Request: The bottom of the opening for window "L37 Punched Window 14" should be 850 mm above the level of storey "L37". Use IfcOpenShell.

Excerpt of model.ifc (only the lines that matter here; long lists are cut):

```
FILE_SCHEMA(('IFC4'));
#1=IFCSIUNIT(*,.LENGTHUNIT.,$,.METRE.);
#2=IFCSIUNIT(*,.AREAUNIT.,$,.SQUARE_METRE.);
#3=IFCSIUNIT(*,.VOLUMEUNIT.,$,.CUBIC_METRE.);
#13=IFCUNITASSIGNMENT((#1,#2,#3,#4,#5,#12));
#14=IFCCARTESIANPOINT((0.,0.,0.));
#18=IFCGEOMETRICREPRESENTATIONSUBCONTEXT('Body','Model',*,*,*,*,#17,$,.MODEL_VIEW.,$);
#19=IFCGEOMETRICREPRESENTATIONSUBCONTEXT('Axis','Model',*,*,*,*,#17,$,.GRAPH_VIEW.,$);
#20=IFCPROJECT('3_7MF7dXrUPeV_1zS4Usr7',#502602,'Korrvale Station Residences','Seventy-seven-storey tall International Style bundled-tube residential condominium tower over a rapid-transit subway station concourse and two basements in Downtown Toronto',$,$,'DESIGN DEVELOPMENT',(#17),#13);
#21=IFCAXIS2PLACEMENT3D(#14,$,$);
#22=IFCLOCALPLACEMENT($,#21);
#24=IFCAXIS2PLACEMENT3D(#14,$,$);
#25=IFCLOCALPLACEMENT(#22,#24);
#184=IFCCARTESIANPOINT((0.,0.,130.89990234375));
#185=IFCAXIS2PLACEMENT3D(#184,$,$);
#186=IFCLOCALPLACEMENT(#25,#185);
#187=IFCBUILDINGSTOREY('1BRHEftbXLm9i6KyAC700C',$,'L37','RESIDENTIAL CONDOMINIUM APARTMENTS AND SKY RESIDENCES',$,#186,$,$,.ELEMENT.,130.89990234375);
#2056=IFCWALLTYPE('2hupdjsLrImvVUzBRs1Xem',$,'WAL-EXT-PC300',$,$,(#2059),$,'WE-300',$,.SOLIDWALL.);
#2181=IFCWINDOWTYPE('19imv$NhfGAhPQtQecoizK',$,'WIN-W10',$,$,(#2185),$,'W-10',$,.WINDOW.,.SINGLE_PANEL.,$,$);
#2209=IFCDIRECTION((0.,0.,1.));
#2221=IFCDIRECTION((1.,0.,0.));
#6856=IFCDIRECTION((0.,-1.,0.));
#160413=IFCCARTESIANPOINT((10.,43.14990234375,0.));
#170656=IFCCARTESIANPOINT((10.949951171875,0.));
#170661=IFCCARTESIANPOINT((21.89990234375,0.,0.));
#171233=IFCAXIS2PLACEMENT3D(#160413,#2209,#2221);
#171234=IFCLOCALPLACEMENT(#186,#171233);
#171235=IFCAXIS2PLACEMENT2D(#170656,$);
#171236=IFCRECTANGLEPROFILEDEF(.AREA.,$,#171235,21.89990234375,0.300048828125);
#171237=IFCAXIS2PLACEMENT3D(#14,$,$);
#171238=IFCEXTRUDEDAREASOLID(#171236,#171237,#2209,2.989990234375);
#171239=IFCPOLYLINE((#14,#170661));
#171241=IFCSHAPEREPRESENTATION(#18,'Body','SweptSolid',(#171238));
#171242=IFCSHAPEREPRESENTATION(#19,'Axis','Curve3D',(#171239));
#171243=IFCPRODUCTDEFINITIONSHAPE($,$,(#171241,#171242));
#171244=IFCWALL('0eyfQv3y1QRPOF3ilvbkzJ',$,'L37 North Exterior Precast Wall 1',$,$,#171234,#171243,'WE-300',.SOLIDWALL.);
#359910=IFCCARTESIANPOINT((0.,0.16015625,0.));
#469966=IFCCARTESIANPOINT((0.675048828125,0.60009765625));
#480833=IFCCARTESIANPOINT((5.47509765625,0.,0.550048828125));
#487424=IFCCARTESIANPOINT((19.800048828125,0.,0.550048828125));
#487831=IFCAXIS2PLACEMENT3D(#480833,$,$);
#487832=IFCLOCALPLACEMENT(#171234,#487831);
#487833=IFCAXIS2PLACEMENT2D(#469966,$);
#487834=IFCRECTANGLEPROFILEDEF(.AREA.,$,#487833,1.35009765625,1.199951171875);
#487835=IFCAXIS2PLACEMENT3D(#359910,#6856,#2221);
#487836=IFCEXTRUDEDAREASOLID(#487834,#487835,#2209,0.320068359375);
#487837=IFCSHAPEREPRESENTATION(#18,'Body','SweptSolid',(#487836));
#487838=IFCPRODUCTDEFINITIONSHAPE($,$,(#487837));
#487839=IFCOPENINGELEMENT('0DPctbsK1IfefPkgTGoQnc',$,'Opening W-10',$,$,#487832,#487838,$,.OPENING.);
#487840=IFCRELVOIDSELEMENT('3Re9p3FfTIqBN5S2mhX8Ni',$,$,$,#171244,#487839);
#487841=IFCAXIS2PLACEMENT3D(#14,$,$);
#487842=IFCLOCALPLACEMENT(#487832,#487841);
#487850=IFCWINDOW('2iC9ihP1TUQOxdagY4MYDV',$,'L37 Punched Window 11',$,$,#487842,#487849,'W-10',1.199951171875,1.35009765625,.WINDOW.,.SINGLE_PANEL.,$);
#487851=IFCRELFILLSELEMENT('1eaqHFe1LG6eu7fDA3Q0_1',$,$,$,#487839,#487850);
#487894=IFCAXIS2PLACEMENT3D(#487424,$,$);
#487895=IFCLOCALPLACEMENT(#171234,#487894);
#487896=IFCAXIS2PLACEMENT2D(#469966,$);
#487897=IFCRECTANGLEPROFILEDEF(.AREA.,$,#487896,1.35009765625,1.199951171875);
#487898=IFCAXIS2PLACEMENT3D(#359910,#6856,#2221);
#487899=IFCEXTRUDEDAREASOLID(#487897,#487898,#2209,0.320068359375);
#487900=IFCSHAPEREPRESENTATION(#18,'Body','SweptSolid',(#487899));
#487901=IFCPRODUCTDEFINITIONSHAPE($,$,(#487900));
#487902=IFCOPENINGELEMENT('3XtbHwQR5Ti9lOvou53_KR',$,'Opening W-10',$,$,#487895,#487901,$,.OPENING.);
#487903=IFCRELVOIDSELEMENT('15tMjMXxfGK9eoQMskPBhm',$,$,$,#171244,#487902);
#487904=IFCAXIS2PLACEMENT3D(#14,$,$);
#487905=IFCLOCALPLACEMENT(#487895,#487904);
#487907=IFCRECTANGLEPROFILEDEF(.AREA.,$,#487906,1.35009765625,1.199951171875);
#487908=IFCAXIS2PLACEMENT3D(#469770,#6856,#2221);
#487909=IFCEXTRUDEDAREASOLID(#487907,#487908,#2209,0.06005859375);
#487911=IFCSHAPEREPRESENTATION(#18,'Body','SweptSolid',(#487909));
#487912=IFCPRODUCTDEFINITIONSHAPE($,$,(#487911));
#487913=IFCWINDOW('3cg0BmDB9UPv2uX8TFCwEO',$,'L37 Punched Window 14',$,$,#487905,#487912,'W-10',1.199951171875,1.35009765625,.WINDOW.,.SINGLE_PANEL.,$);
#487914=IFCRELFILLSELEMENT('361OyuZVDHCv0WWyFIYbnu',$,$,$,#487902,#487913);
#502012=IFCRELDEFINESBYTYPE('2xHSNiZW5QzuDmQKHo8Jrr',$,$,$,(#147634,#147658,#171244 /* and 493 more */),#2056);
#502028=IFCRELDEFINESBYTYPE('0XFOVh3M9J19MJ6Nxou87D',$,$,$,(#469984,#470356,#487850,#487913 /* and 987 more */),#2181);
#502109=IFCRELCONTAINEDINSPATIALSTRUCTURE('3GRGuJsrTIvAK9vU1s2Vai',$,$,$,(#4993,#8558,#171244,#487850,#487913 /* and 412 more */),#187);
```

```python
import numpy as np
import ifcopenshell
import ifcopenshell.api.geometry
import ifcopenshell.geom
import ifcopenshell.util.element
import ifcopenshell.util.placement
import ifcopenshell.util.shape
import ifcopenshell.util.unit

model = ifcopenshell.open("model.ifc")
unit_scale = ifcopenshell.util.unit.calculate_unit_scale(model)

window = model.by_guid("3cg0BmDB9UPv2uX8TFCwEO")
opening = window.FillsVoids[0].RelatingOpeningElement
storey = ifcopenshell.util.element.get_container(window, ifc_class="IfcBuildingStorey")
level = ifcopenshell.util.placement.get_local_placement(storey.ObjectPlacement)[2, 3]

# The opening's origin need not be at the sill, so measure its lowest point.
shape = ifcopenshell.geom.create_shape(ifcopenshell.geom.settings(), opening)
bottom = ifcopenshell.util.shape.get_shape_bottom_elevation(shape, shape.geometry) / unit_scale
dz = level + 0.85 / unit_scale - bottom

shift = np.array([0.0, 0.0, dz])
# The window is placed relative to its opening, so it follows when the opening moves.
matrix = ifcopenshell.util.placement.get_local_placement(opening.ObjectPlacement)
matrix[:3, 3] += shift
ifcopenshell.api.geometry.edit_object_placement(
    model, product=opening, matrix=matrix, is_si=False, should_transform_children=True
)

print(f"moved by {dz * unit_scale:+.3f} m")

model.write("model_edited.ifc")
```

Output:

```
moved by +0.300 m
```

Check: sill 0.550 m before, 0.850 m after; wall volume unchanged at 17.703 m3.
